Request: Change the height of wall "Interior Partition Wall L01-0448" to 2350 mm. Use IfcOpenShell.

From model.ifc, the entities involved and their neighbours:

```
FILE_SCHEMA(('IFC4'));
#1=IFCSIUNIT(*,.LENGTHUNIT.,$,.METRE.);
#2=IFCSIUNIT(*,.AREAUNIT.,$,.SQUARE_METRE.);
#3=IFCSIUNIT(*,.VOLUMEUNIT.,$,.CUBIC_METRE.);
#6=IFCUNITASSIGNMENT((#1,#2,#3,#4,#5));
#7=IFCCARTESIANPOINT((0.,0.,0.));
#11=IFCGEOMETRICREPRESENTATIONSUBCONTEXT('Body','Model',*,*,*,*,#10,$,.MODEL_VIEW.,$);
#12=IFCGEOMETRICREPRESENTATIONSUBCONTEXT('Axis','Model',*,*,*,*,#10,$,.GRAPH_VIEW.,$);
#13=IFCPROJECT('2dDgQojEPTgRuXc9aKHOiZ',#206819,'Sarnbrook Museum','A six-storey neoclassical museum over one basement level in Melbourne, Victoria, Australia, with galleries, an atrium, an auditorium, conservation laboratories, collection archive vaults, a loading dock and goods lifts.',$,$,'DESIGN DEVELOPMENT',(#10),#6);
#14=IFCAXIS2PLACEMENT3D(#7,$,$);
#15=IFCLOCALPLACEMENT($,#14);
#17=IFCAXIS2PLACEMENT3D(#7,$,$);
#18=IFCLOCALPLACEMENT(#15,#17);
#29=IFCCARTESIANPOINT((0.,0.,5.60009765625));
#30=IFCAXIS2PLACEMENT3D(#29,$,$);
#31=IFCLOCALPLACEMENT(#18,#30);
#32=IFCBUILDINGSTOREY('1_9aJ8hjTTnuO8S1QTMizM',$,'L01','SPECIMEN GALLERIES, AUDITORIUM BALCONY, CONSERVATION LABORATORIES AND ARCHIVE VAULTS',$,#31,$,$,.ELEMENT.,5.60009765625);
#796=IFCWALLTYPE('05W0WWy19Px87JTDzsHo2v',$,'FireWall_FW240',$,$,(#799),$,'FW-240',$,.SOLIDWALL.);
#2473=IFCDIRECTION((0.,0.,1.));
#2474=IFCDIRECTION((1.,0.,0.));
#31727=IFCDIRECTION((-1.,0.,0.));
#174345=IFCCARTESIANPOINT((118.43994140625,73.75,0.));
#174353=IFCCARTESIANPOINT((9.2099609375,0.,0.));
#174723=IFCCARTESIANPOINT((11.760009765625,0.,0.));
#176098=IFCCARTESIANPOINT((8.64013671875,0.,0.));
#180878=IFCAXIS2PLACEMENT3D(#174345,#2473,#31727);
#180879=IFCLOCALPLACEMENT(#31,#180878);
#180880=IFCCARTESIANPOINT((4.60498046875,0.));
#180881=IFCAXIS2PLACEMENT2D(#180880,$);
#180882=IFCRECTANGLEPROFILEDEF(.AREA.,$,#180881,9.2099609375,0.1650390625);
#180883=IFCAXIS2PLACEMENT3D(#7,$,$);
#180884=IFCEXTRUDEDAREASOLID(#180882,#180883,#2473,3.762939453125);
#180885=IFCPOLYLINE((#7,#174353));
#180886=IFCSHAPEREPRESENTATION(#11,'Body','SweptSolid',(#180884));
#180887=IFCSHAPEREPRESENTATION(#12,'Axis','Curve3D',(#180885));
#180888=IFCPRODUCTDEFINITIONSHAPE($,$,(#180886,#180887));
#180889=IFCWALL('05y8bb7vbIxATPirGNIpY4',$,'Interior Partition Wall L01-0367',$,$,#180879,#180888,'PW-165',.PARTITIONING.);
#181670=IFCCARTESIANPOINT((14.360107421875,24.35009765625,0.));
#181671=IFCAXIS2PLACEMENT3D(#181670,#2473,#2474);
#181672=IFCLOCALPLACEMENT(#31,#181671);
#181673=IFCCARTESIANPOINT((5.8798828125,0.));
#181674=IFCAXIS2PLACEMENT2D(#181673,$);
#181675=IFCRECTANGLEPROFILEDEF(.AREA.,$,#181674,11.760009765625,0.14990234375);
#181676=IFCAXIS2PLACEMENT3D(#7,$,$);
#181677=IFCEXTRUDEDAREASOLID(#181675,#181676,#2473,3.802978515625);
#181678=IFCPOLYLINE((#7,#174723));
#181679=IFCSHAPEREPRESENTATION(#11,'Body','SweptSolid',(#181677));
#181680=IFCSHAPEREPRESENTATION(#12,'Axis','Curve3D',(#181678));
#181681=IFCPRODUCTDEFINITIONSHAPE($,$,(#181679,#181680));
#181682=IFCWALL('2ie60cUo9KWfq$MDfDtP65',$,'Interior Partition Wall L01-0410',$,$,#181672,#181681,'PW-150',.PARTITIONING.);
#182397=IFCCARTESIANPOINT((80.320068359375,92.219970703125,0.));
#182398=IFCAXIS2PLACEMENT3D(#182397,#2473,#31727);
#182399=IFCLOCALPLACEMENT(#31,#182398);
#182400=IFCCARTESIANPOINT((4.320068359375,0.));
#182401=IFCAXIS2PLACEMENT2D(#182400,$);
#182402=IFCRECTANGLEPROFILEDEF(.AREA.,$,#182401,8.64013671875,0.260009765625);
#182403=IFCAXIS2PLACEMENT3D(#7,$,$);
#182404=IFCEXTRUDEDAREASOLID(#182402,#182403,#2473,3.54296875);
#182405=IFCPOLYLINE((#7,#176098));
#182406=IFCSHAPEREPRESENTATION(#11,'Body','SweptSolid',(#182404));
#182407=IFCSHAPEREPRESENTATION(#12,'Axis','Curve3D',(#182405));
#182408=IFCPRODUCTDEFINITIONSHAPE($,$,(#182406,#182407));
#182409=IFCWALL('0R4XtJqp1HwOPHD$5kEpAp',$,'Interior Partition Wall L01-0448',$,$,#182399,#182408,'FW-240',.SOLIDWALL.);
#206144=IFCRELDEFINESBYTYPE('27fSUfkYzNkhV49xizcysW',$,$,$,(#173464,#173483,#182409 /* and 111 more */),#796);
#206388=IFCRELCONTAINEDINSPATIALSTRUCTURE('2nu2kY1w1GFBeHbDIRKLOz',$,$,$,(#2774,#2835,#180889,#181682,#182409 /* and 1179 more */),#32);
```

```python
import ifcopenshell
import ifcopenshell.geom
import ifcopenshell.util.representation
import ifcopenshell.util.shape

model = ifcopenshell.open("model.ifc")
settings = ifcopenshell.geom.settings()


def volume(element):
    """Net volume in cubic metres, openings subtracted."""
    shape = ifcopenshell.geom.create_shape(settings, element)
    return ifcopenshell.util.shape.get_volume(shape.geometry)


wall = model.by_id(182409)
before = volume(wall)

body = ifcopenshell.util.representation.get_representation(wall, "Model", "Body")
solid = body.Items[0]
old_height = solid.Depth
solid.Depth = 2.35
after = volume(wall)

print(f"height {old_height:g} -> {solid.Depth:g}, volume {before:.3f} -> {after:.3f} m3")

model.write("model-out.ifc")
```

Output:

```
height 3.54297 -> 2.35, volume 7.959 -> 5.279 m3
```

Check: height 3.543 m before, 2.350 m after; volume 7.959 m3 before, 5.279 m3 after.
